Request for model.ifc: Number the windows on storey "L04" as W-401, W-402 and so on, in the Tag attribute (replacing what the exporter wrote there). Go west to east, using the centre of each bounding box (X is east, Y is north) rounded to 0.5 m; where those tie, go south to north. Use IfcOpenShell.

First a look at what the model holds.

```python
import ifcopenshell
import ifcopenshell.util.element
import ifcopenshell.util.placement

model = ifcopenshell.open("model.ifc")
print(model.schema)
storey = next(s for s in model.by_type("IfcBuildingStorey") if s.Name == "L04")
windows = [e for e in ifcopenshell.util.element.get_decomposition(storey) if e.is_a("IfcWindow")]
for e in sorted(windows, key=lambda e: e.id()):
    origin = ifcopenshell.util.placement.get_local_placement(e.ObjectPlacement)[:3, 3]
    print(e.id(), e.Tag, e.Name, origin.round(2) + 0.0, sep=" | ")
```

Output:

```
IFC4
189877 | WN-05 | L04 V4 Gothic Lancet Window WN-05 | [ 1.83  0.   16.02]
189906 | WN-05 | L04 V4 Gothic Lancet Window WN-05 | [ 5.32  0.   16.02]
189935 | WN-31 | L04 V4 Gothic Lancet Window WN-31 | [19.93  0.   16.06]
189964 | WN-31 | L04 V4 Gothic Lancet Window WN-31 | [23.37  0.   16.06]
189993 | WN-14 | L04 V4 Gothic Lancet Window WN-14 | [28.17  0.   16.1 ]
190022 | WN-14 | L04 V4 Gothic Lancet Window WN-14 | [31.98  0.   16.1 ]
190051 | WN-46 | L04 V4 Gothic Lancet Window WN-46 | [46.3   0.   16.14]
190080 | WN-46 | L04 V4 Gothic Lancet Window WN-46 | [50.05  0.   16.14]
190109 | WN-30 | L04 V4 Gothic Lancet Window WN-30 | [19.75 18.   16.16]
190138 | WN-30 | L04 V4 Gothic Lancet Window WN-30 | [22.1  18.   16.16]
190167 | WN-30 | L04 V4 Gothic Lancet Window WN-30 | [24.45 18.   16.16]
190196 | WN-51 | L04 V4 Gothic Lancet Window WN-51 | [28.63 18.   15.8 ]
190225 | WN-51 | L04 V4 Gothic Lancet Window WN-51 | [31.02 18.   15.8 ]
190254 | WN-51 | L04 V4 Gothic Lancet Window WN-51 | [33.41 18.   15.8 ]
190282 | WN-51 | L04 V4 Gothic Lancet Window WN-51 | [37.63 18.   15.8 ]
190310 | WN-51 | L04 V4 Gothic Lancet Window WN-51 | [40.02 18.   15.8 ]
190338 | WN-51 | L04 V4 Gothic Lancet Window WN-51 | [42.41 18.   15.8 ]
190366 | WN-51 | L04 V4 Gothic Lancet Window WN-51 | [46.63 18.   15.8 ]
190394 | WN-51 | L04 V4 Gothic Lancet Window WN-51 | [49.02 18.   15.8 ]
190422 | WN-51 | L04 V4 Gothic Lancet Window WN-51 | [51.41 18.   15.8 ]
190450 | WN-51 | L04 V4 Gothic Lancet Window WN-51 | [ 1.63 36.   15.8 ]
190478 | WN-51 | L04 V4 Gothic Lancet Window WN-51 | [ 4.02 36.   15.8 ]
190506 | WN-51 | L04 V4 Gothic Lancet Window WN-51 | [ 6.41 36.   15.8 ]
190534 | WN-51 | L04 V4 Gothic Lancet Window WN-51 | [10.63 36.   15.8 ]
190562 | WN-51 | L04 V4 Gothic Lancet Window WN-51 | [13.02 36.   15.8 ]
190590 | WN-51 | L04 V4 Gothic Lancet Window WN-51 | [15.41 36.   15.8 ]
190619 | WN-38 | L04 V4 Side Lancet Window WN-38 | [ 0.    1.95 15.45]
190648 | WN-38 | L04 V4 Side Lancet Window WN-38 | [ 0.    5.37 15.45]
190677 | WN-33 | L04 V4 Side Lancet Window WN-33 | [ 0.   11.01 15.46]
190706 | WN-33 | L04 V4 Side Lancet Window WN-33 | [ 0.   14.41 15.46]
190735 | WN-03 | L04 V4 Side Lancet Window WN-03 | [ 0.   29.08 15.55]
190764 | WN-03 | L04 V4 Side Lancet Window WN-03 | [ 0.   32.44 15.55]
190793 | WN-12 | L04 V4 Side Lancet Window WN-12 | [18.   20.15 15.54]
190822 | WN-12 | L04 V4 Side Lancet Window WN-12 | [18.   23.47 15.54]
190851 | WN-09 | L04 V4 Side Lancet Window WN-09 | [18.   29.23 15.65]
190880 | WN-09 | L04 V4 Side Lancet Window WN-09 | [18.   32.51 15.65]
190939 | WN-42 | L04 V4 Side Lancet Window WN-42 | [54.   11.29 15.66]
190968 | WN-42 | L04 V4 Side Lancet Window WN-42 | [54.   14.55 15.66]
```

```python
import ifcopenshell
import ifcopenshell.geom
import ifcopenshell.util.element
import ifcopenshell.util.shape

model = ifcopenshell.open("model.ifc")
settings = ifcopenshell.geom.settings()
settings.set("use-world-coords", True)


def centre(element):
    shape = ifcopenshell.geom.create_shape(settings, element)
    return ifcopenshell.util.shape.get_bbox_centroid(shape.geometry)


storey = next(s for s in model.by_type("IfcBuildingStorey") if s.Name == "L04")
windows = [e for e in ifcopenshell.util.element.get_decomposition(storey) if e.is_a("IfcWindow")]

# Insertion points can sit at a corner or the storey origin, so sort by the geometry (in metres).
centres = {e: centre(e) for e in windows}
windows.sort(key=lambda e: (round(centres[e][0] / 0.5), centres[e][1]))

for i, e in enumerate(windows, start=1):
    number = f"W-4{i:02d}"
    e.Tag = number
    print(e.id(), number)

model.write("model_updated.ifc")
```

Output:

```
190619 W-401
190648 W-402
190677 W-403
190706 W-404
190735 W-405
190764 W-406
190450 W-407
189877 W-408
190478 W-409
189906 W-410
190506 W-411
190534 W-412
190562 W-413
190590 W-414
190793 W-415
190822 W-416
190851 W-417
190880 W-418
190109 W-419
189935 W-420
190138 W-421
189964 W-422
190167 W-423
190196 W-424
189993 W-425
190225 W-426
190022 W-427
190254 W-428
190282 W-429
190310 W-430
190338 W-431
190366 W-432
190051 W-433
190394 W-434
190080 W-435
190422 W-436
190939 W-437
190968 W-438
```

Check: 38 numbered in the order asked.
